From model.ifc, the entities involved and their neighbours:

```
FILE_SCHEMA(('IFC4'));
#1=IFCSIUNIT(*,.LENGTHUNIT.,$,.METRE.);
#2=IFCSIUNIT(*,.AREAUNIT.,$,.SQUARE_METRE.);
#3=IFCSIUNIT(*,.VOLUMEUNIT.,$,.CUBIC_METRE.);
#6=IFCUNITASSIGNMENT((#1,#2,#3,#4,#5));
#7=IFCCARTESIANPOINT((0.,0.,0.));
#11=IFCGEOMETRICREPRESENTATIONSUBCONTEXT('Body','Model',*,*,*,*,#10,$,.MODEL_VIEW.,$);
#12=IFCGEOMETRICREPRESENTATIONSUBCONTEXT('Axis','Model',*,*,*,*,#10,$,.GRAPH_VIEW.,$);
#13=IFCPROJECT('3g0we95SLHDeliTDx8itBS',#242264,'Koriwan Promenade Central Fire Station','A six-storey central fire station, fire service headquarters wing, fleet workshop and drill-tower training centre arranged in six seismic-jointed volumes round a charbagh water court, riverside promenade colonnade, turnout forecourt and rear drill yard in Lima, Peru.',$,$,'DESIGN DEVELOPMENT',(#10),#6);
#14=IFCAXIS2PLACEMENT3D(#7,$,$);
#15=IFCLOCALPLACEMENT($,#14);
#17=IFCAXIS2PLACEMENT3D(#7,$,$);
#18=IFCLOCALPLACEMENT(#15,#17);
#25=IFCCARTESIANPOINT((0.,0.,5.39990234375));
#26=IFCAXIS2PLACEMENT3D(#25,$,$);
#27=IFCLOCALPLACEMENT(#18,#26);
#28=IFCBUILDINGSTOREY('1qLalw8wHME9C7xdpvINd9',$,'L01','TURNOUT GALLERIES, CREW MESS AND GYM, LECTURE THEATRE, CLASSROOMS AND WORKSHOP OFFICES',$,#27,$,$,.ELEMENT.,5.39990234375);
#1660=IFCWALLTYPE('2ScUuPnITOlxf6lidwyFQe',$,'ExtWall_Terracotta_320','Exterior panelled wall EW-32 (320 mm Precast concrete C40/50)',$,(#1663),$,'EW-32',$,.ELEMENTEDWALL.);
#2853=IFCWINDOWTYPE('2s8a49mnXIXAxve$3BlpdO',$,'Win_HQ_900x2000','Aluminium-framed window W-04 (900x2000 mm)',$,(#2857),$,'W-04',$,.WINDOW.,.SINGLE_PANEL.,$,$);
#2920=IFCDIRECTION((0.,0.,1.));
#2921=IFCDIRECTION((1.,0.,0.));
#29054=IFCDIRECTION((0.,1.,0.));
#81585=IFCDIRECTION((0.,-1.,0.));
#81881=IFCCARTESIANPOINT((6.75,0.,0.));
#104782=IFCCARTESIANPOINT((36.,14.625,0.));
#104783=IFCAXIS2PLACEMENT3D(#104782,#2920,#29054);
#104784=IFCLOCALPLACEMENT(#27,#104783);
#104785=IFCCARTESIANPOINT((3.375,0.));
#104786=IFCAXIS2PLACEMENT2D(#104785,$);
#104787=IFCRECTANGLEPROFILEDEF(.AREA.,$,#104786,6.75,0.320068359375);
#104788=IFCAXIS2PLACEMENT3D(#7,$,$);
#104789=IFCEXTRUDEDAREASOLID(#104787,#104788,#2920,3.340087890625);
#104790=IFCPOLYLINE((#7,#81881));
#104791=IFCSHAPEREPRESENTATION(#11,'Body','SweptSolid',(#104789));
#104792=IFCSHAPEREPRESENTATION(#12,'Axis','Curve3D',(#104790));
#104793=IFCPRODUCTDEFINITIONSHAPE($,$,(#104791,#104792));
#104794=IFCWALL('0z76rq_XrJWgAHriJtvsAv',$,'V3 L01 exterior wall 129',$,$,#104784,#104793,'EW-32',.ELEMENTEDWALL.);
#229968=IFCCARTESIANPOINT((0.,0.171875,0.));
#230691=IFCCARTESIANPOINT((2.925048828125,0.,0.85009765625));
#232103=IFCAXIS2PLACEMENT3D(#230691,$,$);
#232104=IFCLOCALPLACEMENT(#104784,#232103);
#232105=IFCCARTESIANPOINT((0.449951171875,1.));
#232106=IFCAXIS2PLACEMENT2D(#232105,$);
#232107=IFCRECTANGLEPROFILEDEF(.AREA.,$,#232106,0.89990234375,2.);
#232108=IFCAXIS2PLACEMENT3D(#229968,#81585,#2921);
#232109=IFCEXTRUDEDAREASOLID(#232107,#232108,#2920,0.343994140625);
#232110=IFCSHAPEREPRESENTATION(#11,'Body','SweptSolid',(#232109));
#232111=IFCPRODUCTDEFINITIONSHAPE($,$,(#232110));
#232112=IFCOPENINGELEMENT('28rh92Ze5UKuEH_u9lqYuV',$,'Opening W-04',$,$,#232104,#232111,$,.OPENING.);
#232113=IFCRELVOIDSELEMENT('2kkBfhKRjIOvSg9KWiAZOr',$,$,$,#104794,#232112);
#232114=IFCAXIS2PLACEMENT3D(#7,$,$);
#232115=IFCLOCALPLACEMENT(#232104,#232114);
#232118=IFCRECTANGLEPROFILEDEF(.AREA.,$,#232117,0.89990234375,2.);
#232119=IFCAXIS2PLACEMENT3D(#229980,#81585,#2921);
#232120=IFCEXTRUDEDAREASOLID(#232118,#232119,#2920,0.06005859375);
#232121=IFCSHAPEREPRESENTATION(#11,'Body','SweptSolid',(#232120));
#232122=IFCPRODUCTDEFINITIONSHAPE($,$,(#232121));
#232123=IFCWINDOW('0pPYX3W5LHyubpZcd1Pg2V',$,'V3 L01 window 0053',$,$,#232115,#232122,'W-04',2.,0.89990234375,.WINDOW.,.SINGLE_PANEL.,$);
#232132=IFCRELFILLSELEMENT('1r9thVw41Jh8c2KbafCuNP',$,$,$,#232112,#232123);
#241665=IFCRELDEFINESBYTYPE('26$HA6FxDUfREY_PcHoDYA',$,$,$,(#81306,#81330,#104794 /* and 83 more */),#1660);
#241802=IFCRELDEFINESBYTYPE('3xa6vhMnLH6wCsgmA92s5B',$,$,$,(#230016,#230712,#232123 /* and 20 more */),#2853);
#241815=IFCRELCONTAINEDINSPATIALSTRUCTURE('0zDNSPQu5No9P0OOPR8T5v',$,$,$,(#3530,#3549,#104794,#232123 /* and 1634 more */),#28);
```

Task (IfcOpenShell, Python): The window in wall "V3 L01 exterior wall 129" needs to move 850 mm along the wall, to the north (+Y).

```python
import ifcopenshell
import ifcopenshell.api.geometry
import ifcopenshell.util.placement
import ifcopenshell.util.unit

model = ifcopenshell.open("model.ifc")
unit_scale = ifcopenshell.util.unit.calculate_unit_scale(model)

window = model.by_id(232123)
opening = window.FillsVoids[0].RelatingOpeningElement
wall = opening.VoidsElements[0].RelatingBuildingElement

wall_matrix = ifcopenshell.util.placement.get_local_placement(wall.ObjectPlacement)
shift = wall_matrix[:3, 0] * 0.85 / unit_scale
before = ifcopenshell.util.placement.get_local_placement(window.ObjectPlacement)[:3, 3].copy()

# The window is placed relative to its opening, so it follows when the opening moves.
matrix = ifcopenshell.util.placement.get_local_placement(opening.ObjectPlacement)
matrix[:3, 3] += shift
ifcopenshell.api.geometry.edit_object_placement(
    model, product=opening, matrix=matrix, is_si=False, should_transform_children=True
)

after = ifcopenshell.util.placement.get_local_placement(window.ObjectPlacement)[:3, 3]
print("window moved by", (after - before).round(3) + 0.0)

model.write("model_updated.ifc")
```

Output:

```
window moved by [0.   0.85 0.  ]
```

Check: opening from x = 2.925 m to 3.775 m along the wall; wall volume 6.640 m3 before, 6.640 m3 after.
